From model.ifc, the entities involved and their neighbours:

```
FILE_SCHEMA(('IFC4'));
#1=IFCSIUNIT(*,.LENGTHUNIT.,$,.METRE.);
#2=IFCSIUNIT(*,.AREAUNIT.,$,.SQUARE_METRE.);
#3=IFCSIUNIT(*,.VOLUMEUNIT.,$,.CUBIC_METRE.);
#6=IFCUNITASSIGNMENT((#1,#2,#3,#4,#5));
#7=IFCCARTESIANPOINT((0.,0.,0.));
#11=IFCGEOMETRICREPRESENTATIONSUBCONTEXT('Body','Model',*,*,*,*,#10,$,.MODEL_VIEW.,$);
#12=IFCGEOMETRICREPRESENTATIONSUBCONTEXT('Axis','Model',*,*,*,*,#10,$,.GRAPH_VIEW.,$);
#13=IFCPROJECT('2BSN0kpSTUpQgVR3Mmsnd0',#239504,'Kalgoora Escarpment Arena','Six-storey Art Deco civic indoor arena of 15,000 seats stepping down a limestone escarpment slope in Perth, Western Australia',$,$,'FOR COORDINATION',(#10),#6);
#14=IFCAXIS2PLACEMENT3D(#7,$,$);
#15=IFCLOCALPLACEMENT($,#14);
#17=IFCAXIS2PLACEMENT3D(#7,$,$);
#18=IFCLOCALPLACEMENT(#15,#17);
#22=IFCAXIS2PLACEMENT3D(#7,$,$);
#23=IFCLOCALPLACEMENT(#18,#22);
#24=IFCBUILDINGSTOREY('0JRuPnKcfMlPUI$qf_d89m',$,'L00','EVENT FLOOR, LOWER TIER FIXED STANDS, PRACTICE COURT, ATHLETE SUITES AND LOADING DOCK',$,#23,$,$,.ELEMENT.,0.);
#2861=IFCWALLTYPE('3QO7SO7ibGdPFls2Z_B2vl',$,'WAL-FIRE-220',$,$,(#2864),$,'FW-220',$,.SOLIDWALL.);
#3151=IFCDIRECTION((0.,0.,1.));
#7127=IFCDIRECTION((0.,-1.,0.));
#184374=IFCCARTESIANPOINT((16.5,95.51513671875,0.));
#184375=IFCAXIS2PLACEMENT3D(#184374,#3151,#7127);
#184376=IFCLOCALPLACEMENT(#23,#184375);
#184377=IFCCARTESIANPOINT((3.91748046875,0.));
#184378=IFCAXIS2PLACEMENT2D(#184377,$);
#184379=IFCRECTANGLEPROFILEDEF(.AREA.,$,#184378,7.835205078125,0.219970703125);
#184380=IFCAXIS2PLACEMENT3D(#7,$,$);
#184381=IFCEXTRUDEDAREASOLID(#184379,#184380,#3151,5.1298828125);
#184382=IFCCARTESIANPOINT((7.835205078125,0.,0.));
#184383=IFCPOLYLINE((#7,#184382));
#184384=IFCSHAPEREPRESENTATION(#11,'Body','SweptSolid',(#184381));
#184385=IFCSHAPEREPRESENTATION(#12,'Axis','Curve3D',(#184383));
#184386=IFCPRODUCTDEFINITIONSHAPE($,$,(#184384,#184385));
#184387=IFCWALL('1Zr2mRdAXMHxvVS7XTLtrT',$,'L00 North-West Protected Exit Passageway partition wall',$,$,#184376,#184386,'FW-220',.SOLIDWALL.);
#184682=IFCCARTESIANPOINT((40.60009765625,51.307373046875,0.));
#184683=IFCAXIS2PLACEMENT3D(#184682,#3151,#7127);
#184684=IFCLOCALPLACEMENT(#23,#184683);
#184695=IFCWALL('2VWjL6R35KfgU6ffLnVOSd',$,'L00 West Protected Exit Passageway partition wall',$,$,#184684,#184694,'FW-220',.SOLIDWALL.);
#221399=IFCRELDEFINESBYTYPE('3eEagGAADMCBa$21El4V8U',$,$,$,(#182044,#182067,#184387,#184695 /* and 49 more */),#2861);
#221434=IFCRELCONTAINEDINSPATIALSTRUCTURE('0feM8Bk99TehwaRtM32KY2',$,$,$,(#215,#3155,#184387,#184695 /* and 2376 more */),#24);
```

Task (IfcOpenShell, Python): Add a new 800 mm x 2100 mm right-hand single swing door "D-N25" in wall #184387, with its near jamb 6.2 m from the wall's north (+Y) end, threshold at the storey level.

```python
import numpy as np
import ifcopenshell
import ifcopenshell.api.feature
import ifcopenshell.api.geometry
import ifcopenshell.api.root
import ifcopenshell.api.spatial
import ifcopenshell.geom
import ifcopenshell.util.element
import ifcopenshell.util.placement
import ifcopenshell.util.representation
import ifcopenshell.util.shape
import ifcopenshell.util.unit

model = ifcopenshell.open("model.ifc")
unit_scale = ifcopenshell.util.unit.calculate_unit_scale(model)
settings = ifcopenshell.geom.settings()


def volume(element):
    """Net volume in cubic metres, openings subtracted."""
    shape = ifcopenshell.geom.create_shape(settings, element)
    return ifcopenshell.util.shape.get_volume(shape.geometry)


wall = model.by_id(184387)
storey = ifcopenshell.util.element.get_container(wall, ifc_class="IfcBuildingStorey")
context = ifcopenshell.util.representation.get_context(model, "Model", "Body", "MODEL_VIEW")
before = volume(wall)

width, height, from_end, sill = 0.8, 2.1, 6.2, 0.0  # metres

# The wall runs along its own X axis, and the end named is its -X end.
wall_shape = ifcopenshell.geom.create_shape(settings, wall)
x, y, z = ifcopenshell.util.shape.get_vertices(wall_shape.geometry).T
start = x.min() + from_end
face, thickness = float(y.min()), float(y.max() - y.min())
wall_matrix = ifcopenshell.util.placement.get_local_placement(wall.ObjectPlacement)
level = ifcopenshell.util.placement.get_local_placement(storey.ObjectPlacement)[2, 3]


def in_wall(x, y):
    """Placement at x, y metres in the wall's axes, at sill height."""
    matrix = wall_matrix.copy()
    matrix[:, 3] = wall_matrix @ np.array([x / unit_scale, y / unit_scale, 0.0, 1.0])
    matrix[2, 3] = level + sill / unit_scale
    return matrix


# Opening: a box that overshoots both wall faces by 50 mm.
opening = ifcopenshell.api.root.create_entity(model, ifc_class="IfcOpeningElement", predefined_type="OPENING")
box = ifcopenshell.api.geometry.add_wall_representation(
    model, context=context, length=width, height=height, thickness=thickness + 0.1
)
ifcopenshell.api.geometry.assign_representation(model, product=opening, representation=box)
ifcopenshell.api.geometry.edit_object_placement(model, product=opening, matrix=in_wall(start, face - 0.05), is_si=False)
ifcopenshell.api.feature.add_feature(model, feature=opening, element=wall)

door = ifcopenshell.api.root.create_entity(model, ifc_class="IfcDoor", name="D-N25", predefined_type="DOOR")
door.OverallWidth, door.OverallHeight = width / unit_scale, height / unit_scale
door.OperationType = "SINGLE_SWING_RIGHT"
body = ifcopenshell.api.geometry.add_door_representation(
    model,
    context=context,
    overall_width=door.OverallWidth,
    overall_height=door.OverallHeight,
    operation_type="SINGLE_SWING_RIGHT",
    lining_properties={"LiningDepth": thickness / unit_scale, "ThresholdDepth": thickness / unit_scale},
)
ifcopenshell.api.geometry.assign_representation(model, product=door, representation=body)
ifcopenshell.api.spatial.assign_container(model, products=[door], relating_structure=storey)
ifcopenshell.api.feature.add_filling(model, opening=opening, element=door)

# The lining spans the wall, so the door starts at the wall face.
ifcopenshell.api.geometry.edit_object_placement(model, product=door, matrix=in_wall(start, face), is_si=False)

after = volume(wall)

print(f"wall volume {before:.3f} -> {after:.3f} m3")

model.write("model-out.ifc")
```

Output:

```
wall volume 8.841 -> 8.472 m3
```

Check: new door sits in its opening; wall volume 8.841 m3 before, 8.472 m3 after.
